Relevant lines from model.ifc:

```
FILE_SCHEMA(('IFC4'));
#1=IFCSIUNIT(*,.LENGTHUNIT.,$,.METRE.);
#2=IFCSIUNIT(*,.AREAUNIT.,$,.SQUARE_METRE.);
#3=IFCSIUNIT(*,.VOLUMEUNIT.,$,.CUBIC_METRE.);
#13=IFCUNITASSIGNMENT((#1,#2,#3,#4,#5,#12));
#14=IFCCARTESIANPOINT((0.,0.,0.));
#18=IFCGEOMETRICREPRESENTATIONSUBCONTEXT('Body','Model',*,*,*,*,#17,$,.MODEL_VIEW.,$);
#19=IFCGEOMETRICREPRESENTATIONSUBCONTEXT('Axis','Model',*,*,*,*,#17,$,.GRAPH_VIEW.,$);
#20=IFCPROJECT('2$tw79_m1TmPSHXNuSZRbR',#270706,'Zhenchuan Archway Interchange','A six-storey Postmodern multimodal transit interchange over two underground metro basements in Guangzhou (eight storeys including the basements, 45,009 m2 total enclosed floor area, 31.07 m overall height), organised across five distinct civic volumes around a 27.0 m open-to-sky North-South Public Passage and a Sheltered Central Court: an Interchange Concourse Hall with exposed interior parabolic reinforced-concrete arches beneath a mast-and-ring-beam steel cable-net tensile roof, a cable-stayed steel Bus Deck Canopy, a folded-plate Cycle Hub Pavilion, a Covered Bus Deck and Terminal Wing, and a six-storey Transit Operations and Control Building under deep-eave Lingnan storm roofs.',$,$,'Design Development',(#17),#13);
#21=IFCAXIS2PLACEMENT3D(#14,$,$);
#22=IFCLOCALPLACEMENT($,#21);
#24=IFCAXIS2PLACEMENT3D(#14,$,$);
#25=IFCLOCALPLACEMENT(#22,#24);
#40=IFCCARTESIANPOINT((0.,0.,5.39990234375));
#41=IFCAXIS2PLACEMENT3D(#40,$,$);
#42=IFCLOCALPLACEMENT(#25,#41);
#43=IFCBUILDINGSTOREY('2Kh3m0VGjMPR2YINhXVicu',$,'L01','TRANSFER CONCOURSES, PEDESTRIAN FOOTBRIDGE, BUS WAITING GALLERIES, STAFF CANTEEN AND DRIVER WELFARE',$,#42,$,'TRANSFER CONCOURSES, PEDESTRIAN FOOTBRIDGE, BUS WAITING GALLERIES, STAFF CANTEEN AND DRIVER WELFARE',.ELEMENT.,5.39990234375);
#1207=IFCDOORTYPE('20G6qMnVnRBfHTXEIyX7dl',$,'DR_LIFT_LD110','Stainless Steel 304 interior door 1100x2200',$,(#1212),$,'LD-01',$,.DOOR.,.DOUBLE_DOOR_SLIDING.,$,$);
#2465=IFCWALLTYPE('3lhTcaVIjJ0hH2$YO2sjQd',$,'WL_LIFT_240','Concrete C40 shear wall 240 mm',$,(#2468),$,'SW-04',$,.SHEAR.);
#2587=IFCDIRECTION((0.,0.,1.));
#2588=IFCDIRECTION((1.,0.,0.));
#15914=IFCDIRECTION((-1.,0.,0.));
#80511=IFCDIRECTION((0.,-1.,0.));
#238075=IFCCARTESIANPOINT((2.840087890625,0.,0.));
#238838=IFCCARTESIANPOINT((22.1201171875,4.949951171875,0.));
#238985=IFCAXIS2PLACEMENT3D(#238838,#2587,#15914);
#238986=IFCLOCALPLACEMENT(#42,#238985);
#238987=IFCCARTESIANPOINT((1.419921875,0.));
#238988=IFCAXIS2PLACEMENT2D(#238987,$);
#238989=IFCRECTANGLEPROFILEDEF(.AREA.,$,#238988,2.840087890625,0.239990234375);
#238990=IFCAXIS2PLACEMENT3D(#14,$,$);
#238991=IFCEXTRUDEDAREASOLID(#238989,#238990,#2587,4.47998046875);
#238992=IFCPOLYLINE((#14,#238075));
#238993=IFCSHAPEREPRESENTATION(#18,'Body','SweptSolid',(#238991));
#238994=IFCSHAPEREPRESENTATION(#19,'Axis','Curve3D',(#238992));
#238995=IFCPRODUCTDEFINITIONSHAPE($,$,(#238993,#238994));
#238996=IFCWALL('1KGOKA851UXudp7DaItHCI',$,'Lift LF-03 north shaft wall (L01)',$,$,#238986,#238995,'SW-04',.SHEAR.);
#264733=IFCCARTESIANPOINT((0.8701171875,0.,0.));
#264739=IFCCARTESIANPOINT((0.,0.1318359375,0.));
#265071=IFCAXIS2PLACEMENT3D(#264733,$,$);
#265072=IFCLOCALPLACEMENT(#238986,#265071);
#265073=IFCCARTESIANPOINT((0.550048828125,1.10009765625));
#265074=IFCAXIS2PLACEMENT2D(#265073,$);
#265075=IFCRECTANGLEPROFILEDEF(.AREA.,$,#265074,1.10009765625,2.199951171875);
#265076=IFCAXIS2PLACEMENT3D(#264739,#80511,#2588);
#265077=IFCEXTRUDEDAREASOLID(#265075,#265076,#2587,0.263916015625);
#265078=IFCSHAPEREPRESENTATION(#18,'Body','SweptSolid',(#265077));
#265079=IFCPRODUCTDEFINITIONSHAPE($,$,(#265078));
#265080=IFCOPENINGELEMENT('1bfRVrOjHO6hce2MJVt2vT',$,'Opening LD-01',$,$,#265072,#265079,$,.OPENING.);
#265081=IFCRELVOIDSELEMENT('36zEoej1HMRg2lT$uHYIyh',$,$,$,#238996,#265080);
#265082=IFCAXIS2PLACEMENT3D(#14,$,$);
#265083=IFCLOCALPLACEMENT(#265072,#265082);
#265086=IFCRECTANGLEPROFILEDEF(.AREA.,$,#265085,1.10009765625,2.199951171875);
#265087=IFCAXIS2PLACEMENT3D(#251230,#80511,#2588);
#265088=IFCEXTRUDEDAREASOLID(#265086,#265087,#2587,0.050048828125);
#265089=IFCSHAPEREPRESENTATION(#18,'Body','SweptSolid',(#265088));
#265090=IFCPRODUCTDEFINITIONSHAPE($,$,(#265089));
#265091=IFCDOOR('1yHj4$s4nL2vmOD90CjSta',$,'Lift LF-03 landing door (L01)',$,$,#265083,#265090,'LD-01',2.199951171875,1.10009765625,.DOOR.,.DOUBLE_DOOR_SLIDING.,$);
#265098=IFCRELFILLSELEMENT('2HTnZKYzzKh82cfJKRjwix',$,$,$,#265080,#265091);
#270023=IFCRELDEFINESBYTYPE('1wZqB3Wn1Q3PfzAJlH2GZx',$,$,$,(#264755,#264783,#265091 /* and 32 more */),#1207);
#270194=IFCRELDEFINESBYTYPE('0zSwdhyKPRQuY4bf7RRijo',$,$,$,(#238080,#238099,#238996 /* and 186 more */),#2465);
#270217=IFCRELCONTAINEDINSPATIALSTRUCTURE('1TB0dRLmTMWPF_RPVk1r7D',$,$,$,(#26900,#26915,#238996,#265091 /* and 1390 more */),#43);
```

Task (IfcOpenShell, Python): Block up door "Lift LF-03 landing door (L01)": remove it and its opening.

```python
import ifcopenshell
import ifcopenshell.api.feature
import ifcopenshell.api.root
import ifcopenshell.geom
import ifcopenshell.util.shape

model = ifcopenshell.open("model.ifc")
settings = ifcopenshell.geom.settings()


def volume(element):
    """Net volume in cubic metres, openings subtracted."""
    shape = ifcopenshell.geom.create_shape(settings, element)
    return ifcopenshell.util.shape.get_volume(shape.geometry)


door = model.by_guid("1yHj4$s4nL2vmOD90CjSta")
opening = door.FillsVoids[0].RelatingOpeningElement
wall = opening.VoidsElements[0].RelatingBuildingElement
before = volume(wall)

ifcopenshell.api.root.remove_product(model, product=door)
ifcopenshell.api.feature.remove_feature(model, feature=opening)

after = volume(wall)

print(f"wall volume {before:.3f} -> {after:.3f} m3")

model.write("model-out.ifc")
```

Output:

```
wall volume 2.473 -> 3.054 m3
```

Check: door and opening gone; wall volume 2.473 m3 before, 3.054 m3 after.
